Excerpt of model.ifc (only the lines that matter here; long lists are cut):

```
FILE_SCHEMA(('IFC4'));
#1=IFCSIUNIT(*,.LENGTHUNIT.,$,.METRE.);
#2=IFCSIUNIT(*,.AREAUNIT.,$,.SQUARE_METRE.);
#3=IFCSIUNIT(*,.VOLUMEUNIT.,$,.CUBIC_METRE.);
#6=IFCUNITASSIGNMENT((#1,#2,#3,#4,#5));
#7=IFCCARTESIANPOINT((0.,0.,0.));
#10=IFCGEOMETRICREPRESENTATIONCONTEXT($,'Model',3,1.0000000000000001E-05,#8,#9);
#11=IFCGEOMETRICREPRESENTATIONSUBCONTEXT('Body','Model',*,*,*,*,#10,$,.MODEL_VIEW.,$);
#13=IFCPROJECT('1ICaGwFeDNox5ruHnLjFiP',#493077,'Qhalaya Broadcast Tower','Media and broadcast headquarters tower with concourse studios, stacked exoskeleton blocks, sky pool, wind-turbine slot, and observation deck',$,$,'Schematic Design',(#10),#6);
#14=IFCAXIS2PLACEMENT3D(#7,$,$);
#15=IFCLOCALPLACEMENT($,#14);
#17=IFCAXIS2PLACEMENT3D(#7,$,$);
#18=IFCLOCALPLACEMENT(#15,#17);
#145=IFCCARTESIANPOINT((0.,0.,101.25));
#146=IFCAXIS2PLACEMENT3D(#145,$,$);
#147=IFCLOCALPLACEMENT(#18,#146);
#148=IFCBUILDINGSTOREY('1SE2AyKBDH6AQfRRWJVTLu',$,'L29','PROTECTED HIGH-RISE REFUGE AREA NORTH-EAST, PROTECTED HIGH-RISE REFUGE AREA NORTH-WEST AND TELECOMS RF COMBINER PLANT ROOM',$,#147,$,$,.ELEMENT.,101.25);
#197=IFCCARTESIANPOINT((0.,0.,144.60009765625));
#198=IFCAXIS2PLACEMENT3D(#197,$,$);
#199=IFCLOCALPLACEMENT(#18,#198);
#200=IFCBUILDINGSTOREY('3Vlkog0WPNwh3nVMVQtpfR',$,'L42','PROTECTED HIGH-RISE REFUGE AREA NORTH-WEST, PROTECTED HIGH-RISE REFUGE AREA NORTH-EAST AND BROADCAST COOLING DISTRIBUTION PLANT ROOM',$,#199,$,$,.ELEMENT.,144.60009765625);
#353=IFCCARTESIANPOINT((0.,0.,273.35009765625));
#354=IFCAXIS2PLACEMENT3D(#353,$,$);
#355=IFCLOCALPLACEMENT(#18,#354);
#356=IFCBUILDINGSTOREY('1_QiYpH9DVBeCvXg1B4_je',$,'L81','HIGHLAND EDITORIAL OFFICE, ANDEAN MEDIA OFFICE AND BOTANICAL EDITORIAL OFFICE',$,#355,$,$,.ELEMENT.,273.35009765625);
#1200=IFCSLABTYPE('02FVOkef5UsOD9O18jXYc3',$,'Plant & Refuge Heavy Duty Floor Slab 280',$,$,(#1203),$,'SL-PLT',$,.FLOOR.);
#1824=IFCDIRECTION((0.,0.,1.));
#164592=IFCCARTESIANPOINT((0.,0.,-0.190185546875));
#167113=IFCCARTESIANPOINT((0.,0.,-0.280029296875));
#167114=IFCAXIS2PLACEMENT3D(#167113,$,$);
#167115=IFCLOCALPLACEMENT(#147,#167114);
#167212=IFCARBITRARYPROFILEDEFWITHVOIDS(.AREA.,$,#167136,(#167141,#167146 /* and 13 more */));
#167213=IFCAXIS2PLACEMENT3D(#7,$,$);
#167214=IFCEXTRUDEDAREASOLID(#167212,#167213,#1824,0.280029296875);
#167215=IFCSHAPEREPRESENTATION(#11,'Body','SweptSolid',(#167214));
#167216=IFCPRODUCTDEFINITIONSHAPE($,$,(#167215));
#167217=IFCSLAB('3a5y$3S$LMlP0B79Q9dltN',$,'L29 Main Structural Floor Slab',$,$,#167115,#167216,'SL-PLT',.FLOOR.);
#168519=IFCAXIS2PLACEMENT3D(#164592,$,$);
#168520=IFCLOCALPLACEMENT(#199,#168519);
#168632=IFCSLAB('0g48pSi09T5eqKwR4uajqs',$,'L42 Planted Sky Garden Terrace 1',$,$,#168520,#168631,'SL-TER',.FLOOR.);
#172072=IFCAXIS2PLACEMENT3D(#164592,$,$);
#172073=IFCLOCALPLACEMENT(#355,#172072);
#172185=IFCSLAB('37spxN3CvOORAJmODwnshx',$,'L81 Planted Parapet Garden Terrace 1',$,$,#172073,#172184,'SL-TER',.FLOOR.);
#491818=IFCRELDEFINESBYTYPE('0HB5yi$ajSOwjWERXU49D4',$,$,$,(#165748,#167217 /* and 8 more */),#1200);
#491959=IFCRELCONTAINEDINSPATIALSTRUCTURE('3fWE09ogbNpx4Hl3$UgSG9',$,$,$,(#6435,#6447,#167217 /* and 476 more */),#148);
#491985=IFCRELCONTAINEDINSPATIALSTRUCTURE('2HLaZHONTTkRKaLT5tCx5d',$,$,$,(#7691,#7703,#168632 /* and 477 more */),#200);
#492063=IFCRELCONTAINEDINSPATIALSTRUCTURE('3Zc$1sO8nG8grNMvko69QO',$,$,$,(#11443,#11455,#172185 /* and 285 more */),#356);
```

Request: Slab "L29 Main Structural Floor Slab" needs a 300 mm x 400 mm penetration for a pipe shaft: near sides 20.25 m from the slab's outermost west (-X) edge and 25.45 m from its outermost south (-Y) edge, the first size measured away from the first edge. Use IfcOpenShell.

```python
import numpy as np
import ifcopenshell
import ifcopenshell.api.feature
import ifcopenshell.api.geometry
import ifcopenshell.api.root
import ifcopenshell.geom
import ifcopenshell.util.placement
import ifcopenshell.util.representation
import ifcopenshell.util.shape
import ifcopenshell.util.unit

model = ifcopenshell.open("model.ifc")
unit_scale = ifcopenshell.util.unit.calculate_unit_scale(model)
settings = ifcopenshell.geom.settings()


def volume(element):
    """Net volume in cubic metres, openings subtracted."""
    shape = ifcopenshell.geom.create_shape(settings, element)
    return ifcopenshell.util.shape.get_volume(shape.geometry)


slab = model.by_guid("3a5y$3S$LMlP0B79Q9dltN")
before = volume(slab)

# Extent in the slab's own axes, in metres. The edges named are its -X and -Y sides.
slab_shape = ifcopenshell.geom.create_shape(settings, slab)
vertices = ifcopenshell.util.shape.get_vertices(slab_shape.geometry)
x_min, y_min, bottom = vertices.min(axis=0)
top = vertices[:, 2].max()

opening = ifcopenshell.api.root.create_entity(model, ifc_class="IfcOpeningElement", name="Pipe shaft opening", predefined_type="OPENING")
context = ifcopenshell.util.representation.get_context(model, "Model", "Body", "MODEL_VIEW")
width, depth = 0.3, 0.4
outline = [(0.0, 0.0), (width, 0.0), (width, depth), (0.0, depth), (0.0, 0.0)]
# Overshoot both faces by 50 mm so the cut is clean.
shape = ifcopenshell.api.geometry.add_slab_representation(
    model, context=context, depth=top - bottom + 0.1, polyline=outline
)
ifcopenshell.api.geometry.assign_representation(model, product=opening, representation=shape)

matrix = ifcopenshell.util.placement.get_local_placement(slab.ObjectPlacement)
matrix[:, 3] = matrix @ np.append(np.array([x_min + 20.25, y_min + 25.45, bottom - 0.05]) / unit_scale, 1.0)
ifcopenshell.api.geometry.edit_object_placement(model, product=opening, matrix=matrix, is_si=False)
ifcopenshell.api.feature.add_feature(model, feature=opening, element=slab)

after = volume(slab)

print(f"slab volume {before:.3f} -> {after:.3f} m3")

model.write("model_rev.ifc")
```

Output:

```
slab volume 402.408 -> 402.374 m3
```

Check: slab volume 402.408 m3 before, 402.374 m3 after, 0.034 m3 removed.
